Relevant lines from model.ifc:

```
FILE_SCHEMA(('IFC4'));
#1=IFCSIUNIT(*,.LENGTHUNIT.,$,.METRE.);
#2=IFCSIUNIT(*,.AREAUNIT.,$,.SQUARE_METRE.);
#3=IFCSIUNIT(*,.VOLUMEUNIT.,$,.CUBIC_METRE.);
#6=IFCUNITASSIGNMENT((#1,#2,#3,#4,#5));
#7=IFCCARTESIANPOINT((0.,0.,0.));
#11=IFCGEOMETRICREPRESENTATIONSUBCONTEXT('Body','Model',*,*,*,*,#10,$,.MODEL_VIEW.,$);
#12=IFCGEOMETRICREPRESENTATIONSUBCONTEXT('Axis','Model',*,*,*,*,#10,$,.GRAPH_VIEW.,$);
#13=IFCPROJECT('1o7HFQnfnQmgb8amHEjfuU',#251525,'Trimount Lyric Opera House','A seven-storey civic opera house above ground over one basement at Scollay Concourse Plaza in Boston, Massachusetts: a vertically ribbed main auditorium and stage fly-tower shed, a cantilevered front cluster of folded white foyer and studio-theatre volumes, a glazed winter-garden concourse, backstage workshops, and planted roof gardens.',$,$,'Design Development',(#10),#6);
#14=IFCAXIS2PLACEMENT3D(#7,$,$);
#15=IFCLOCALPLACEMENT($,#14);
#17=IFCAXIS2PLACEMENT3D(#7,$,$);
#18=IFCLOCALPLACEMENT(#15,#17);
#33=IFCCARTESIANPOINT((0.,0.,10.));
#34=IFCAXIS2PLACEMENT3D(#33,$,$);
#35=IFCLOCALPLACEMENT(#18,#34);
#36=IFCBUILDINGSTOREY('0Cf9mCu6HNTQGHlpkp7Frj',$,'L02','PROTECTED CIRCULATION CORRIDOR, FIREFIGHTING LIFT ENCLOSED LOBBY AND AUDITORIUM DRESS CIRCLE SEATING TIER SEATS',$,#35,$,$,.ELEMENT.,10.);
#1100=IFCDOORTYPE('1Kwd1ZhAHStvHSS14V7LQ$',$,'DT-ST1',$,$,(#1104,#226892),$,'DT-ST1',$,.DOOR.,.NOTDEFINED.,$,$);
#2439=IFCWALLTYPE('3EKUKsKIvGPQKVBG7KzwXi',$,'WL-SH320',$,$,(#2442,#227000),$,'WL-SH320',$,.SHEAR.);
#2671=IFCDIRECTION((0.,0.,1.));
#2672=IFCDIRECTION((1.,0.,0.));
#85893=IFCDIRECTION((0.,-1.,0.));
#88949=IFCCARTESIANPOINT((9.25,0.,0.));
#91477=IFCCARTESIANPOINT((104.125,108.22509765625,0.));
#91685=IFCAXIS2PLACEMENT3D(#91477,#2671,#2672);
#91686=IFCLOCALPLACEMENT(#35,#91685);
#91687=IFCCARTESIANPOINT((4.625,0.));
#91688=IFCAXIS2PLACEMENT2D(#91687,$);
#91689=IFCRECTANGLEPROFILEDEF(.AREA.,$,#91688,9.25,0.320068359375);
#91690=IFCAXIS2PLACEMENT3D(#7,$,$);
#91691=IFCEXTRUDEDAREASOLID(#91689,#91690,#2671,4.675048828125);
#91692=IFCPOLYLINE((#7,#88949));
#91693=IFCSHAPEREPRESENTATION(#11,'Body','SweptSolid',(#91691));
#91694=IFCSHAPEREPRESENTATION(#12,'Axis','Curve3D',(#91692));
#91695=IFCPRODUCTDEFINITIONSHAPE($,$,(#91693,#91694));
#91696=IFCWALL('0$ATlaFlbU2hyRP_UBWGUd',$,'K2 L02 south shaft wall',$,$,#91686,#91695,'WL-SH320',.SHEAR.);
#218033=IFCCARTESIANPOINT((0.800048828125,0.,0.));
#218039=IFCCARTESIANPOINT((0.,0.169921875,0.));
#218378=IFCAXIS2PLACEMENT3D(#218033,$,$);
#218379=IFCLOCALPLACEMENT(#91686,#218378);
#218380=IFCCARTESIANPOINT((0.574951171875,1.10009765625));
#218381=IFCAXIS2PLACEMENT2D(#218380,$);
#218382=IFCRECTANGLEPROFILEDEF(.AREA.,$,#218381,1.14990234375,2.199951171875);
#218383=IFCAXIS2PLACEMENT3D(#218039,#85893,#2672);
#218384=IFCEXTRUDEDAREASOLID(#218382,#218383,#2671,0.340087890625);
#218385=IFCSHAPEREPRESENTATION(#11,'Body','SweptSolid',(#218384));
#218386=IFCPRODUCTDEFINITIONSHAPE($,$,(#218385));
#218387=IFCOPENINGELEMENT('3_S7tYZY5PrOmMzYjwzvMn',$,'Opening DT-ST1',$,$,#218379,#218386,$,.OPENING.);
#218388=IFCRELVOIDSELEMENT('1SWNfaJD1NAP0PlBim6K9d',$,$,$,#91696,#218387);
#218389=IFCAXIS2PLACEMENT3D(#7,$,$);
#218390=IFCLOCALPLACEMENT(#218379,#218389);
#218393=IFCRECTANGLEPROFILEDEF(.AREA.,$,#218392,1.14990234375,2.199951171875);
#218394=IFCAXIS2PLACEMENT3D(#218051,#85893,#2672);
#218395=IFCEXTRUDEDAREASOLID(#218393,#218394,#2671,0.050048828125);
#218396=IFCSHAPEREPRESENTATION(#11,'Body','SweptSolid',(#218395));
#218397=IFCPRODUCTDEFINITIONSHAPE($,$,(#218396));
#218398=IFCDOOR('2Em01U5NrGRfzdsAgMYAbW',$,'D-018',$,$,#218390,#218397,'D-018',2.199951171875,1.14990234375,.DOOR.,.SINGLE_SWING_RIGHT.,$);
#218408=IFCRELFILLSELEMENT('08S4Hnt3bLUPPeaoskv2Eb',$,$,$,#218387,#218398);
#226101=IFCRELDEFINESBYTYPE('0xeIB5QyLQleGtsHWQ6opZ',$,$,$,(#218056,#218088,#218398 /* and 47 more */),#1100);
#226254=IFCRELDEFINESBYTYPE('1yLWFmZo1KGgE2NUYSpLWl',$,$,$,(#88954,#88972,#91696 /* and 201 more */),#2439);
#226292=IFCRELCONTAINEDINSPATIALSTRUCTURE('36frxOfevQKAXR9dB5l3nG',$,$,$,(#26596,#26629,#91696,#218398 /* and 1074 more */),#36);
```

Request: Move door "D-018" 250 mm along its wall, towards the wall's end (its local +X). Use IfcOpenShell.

```python
import ifcopenshell
import ifcopenshell.api.geometry
import ifcopenshell.util.placement

model = ifcopenshell.open("model.ifc")

door = model.by_guid("2Em01U5NrGRfzdsAgMYAbW")
opening = door.FillsVoids[0].RelatingOpeningElement
wall = opening.VoidsElements[0].RelatingBuildingElement

wall_matrix = ifcopenshell.util.placement.get_local_placement(wall.ObjectPlacement)
shift = wall_matrix[:3, 0] * 0.25
before = ifcopenshell.util.placement.get_local_placement(door.ObjectPlacement)[:3, 3].copy()

# The door is placed relative to its opening, so it follows when the opening moves.
matrix = ifcopenshell.util.placement.get_local_placement(opening.ObjectPlacement)
matrix[:3, 3] += shift
ifcopenshell.api.geometry.edit_object_placement(
    model, product=opening, matrix=matrix, is_si=False, should_transform_children=True
)

after = ifcopenshell.util.placement.get_local_placement(door.ObjectPlacement)[:3, 3]
print("door moved by", (after - before).round(3) + 0.0)

model.write("model_edited.ifc")
```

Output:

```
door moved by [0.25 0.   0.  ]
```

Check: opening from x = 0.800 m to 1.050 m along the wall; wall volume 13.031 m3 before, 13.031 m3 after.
